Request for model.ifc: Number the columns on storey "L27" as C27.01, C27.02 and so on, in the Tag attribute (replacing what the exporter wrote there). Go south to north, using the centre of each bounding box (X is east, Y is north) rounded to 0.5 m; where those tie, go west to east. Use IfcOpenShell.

First a look at what the model holds.

```python
import ifcopenshell
import ifcopenshell.util.element
import ifcopenshell.util.placement

model = ifcopenshell.open("model.ifc")
print(model.schema)
storey = next(s for s in model.by_type("IfcBuildingStorey") if s.Name == "L27")
columns = [e for e in ifcopenshell.util.element.get_decomposition(storey) if e.is_a("IfcColumn")]
for e in sorted(columns, key=lambda e: e.id()):
    origin = ifcopenshell.util.placement.get_local_placement(e.ObjectPlacement)[:3, 3]
    print(e.id(), e.Tag, e.Name, origin.round(2) + 0.0, sep=" | ")
```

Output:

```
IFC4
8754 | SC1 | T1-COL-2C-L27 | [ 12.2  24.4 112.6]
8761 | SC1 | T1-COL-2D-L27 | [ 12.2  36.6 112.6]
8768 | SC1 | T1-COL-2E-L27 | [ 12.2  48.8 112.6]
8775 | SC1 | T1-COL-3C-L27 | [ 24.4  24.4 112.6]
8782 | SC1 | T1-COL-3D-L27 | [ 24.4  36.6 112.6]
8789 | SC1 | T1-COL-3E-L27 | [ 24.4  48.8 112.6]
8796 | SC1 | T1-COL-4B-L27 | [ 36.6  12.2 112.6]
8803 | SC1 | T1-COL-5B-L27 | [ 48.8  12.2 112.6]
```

```python
import ifcopenshell
import ifcopenshell.geom
import ifcopenshell.util.element
import ifcopenshell.util.shape

model = ifcopenshell.open("model.ifc")
settings = ifcopenshell.geom.settings()
settings.set("use-world-coords", True)


def centre(element):
    shape = ifcopenshell.geom.create_shape(settings, element)
    return ifcopenshell.util.shape.get_bbox_centroid(shape.geometry)


storey = next(s for s in model.by_type("IfcBuildingStorey") if s.Name == "L27")
columns = [e for e in ifcopenshell.util.element.get_decomposition(storey) if e.is_a("IfcColumn")]

# Insertion points can sit at a corner or the storey origin, so sort by the geometry (in metres).
centres = {e: centre(e) for e in columns}
columns.sort(key=lambda e: (round(centres[e][1] / 0.5), centres[e][0]))

for i, e in enumerate(columns, start=1):
    number = f"C27.{i:02d}"
    e.Tag = number
    print(e.id(), number)

model.write("model_edited.ifc")
```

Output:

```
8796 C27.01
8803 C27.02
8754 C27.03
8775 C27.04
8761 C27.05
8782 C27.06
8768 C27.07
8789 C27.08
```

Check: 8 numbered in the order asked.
